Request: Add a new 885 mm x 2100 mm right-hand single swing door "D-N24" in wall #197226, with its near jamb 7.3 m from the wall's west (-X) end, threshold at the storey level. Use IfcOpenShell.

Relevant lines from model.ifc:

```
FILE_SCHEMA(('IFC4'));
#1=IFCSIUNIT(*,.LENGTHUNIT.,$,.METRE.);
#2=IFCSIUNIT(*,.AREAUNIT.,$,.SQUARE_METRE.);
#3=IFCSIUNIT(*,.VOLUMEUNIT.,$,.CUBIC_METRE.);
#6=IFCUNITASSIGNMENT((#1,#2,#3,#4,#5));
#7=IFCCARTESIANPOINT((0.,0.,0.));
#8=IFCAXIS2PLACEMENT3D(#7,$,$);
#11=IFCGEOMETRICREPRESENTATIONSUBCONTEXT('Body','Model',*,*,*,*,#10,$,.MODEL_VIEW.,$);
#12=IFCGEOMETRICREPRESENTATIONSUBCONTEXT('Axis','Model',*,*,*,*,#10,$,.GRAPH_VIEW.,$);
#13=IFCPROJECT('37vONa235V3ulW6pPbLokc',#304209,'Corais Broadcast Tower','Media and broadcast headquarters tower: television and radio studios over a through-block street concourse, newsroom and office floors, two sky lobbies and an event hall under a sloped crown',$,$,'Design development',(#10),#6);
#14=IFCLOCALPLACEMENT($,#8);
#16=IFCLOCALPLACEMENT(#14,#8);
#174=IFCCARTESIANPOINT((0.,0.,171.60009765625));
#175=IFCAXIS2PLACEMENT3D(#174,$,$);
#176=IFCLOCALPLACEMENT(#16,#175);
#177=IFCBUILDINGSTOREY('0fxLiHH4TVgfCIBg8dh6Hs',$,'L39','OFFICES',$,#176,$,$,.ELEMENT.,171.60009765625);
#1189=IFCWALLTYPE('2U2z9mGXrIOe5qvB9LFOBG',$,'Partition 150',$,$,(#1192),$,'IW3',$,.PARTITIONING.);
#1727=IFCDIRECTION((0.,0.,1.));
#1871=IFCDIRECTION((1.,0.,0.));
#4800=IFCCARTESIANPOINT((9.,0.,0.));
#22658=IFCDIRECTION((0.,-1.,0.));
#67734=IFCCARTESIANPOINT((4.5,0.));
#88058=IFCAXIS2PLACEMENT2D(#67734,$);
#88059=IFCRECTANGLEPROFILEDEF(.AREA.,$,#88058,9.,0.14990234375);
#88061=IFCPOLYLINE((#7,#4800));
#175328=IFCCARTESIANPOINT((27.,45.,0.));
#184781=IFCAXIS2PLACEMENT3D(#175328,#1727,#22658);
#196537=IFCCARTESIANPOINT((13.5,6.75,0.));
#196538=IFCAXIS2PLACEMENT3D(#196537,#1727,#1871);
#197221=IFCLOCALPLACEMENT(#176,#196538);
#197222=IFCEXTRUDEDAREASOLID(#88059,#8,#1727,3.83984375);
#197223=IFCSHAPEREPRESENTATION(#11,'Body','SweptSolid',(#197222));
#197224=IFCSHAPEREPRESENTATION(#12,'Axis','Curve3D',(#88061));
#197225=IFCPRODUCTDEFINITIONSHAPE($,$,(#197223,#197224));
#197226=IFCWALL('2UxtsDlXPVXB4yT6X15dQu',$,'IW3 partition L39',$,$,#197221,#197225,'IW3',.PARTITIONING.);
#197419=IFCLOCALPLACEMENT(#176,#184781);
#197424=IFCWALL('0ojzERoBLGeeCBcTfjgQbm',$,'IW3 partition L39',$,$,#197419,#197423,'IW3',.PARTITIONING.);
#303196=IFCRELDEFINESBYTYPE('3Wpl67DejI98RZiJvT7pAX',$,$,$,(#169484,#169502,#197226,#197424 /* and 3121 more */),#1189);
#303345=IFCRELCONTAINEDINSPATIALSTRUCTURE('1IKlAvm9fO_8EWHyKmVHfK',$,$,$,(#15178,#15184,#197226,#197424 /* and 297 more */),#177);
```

```python
import numpy as np
import ifcopenshell
import ifcopenshell.api.feature
import ifcopenshell.api.geometry
import ifcopenshell.api.root
import ifcopenshell.api.spatial
import ifcopenshell.geom
import ifcopenshell.util.element
import ifcopenshell.util.placement
import ifcopenshell.util.representation
import ifcopenshell.util.shape
import ifcopenshell.util.unit

model = ifcopenshell.open("model.ifc")
unit_scale = ifcopenshell.util.unit.calculate_unit_scale(model)
settings = ifcopenshell.geom.settings()


def volume(element):
    """Net volume in cubic metres, openings subtracted."""
    shape = ifcopenshell.geom.create_shape(settings, element)
    return ifcopenshell.util.shape.get_volume(shape.geometry)


wall = model.by_guid("2UxtsDlXPVXB4yT6X15dQu")
storey = ifcopenshell.util.element.get_container(wall, ifc_class="IfcBuildingStorey")
context = ifcopenshell.util.representation.get_context(model, "Model", "Body", "MODEL_VIEW")
before = volume(wall)

width, height, from_end, sill = 0.885, 2.1, 7.3, 0.0  # metres

# The wall runs along its own X axis, and the end named is its -X end.
wall_shape = ifcopenshell.geom.create_shape(settings, wall)
x, y, z = ifcopenshell.util.shape.get_vertices(wall_shape.geometry).T
start = x.min() + from_end
face, thickness = float(y.min()), float(y.max() - y.min())
wall_matrix = ifcopenshell.util.placement.get_local_placement(wall.ObjectPlacement)
level = ifcopenshell.util.placement.get_local_placement(storey.ObjectPlacement)[2, 3]


def in_wall(x, y):
    """Placement at x, y metres in the wall's axes, at sill height."""
    matrix = wall_matrix.copy()
    matrix[:, 3] = wall_matrix @ np.array([x / unit_scale, y / unit_scale, 0.0, 1.0])
    matrix[2, 3] = level + sill / unit_scale
    return matrix


# Opening: a box that overshoots both wall faces by 50 mm.
opening = ifcopenshell.api.root.create_entity(model, ifc_class="IfcOpeningElement", predefined_type="OPENING")
box = ifcopenshell.api.geometry.add_wall_representation(
    model, context=context, length=width, height=height, thickness=thickness + 0.1
)
ifcopenshell.api.geometry.assign_representation(model, product=opening, representation=box)
ifcopenshell.api.geometry.edit_object_placement(model, product=opening, matrix=in_wall(start, face - 0.05), is_si=False)
ifcopenshell.api.feature.add_feature(model, feature=opening, element=wall)

door = ifcopenshell.api.root.create_entity(model, ifc_class="IfcDoor", name="D-N24", predefined_type="DOOR")
door.OverallWidth, door.OverallHeight = width / unit_scale, height / unit_scale
door.OperationType = "SINGLE_SWING_RIGHT"
body = ifcopenshell.api.geometry.add_door_representation(
    model,
    context=context,
    overall_width=door.OverallWidth,
    overall_height=door.OverallHeight,
    operation_type="SINGLE_SWING_RIGHT",
    lining_properties={"LiningDepth": thickness / unit_scale, "ThresholdDepth": thickness / unit_scale},
)
ifcopenshell.api.geometry.assign_representation(model, product=door, representation=body)
ifcopenshell.api.spatial.assign_container(model, products=[door], relating_structure=storey)
ifcopenshell.api.feature.add_filling(model, opening=opening, element=door)

# The lining spans the wall, so the door starts at the wall face.
ifcopenshell.api.geometry.edit_object_placement(model, product=door, matrix=in_wall(start, face), is_si=False)

after = volume(wall)

print(f"wall volume {before:.3f} -> {after:.3f} m3")

model.write("model_rev.ifc")
```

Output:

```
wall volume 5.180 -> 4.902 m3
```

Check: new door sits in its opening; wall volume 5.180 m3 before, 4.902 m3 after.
